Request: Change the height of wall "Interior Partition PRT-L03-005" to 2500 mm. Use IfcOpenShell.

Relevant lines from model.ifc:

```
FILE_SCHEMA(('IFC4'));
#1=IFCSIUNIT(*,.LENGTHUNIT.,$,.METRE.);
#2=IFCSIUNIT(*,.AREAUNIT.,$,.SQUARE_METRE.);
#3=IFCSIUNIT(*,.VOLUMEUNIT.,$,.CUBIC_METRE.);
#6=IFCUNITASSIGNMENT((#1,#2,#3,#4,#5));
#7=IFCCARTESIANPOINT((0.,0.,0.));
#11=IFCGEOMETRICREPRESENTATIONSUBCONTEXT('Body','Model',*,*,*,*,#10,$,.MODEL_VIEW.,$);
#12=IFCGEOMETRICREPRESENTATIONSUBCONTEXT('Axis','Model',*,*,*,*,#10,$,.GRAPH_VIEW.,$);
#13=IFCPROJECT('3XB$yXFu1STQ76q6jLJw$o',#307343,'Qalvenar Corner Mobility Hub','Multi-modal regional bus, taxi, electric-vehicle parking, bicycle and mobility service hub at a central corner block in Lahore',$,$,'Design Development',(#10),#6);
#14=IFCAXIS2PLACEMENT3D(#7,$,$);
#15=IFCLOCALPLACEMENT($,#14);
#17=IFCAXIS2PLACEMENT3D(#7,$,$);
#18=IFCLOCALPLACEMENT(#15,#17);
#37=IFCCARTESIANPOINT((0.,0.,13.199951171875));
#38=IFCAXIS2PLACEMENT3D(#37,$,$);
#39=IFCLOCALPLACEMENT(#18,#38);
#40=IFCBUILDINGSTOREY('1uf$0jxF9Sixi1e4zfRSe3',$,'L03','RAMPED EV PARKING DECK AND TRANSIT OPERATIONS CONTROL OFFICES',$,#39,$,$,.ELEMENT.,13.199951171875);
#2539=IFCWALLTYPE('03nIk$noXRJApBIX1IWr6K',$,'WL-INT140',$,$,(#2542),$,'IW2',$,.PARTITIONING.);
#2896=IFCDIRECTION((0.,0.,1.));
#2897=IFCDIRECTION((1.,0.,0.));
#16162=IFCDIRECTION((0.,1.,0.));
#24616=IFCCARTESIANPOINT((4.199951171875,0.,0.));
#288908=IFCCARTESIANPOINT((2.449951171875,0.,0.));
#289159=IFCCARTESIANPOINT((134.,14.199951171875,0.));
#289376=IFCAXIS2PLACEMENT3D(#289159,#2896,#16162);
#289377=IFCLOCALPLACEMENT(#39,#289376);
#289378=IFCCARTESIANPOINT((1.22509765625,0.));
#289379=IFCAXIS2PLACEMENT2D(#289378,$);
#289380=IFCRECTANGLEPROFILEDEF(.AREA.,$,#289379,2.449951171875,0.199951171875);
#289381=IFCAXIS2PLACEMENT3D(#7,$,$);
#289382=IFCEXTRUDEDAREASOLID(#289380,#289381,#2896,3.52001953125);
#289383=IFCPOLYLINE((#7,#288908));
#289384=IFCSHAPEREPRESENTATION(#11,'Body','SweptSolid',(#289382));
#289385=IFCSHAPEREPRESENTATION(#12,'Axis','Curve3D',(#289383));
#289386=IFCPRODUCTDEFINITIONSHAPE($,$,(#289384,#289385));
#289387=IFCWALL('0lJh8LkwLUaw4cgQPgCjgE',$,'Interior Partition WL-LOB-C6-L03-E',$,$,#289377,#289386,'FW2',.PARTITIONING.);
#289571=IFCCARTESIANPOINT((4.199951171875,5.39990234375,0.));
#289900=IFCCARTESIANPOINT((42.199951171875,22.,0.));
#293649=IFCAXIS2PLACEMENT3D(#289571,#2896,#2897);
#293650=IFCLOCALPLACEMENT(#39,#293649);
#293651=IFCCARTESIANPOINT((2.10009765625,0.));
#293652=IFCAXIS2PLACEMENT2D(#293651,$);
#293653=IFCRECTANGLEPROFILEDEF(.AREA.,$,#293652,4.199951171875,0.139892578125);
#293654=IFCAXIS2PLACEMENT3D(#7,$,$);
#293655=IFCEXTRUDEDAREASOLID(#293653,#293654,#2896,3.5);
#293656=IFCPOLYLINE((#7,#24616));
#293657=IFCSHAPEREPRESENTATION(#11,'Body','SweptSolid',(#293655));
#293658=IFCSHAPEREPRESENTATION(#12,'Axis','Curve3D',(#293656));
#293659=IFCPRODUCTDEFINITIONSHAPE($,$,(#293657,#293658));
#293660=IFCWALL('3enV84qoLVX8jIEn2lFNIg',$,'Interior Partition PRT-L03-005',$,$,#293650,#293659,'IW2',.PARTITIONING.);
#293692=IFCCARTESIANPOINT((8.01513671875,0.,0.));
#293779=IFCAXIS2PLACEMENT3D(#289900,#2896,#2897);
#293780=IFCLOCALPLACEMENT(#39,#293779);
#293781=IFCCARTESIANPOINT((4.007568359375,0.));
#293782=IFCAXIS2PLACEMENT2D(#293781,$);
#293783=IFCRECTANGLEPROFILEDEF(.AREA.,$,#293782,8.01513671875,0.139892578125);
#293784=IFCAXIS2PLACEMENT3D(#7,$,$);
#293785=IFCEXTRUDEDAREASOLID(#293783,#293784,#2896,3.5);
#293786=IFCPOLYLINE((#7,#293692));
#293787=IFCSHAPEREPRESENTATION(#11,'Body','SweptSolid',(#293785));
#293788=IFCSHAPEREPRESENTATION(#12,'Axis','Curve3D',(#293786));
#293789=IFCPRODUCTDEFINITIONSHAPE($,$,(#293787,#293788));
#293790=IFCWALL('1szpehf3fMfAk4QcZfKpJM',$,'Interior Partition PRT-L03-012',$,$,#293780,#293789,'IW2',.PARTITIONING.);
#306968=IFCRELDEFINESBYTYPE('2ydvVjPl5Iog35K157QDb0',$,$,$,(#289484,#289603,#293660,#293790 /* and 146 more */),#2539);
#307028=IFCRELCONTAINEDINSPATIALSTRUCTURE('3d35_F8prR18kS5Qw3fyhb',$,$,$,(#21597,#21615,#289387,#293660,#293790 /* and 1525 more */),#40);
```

```python
import ifcopenshell
import ifcopenshell.geom
import ifcopenshell.util.representation
import ifcopenshell.util.shape
import ifcopenshell.util.unit

model = ifcopenshell.open("model.ifc")
unit_scale = ifcopenshell.util.unit.calculate_unit_scale(model)
settings = ifcopenshell.geom.settings()


def volume(element):
    """Net volume in cubic metres, openings subtracted."""
    shape = ifcopenshell.geom.create_shape(settings, element)
    return ifcopenshell.util.shape.get_volume(shape.geometry)


wall = model.by_guid("3enV84qoLVX8jIEn2lFNIg")
before = volume(wall)

body = ifcopenshell.util.representation.get_representation(wall, "Model", "Body")
solid = body.Items[0]
old_height = solid.Depth
solid.Depth = 2.5 / unit_scale
after = volume(wall)

print(f"height {old_height:g} -> {solid.Depth:g}, volume {before:.3f} -> {after:.3f} m3")

model.write("model_edited.ifc")
```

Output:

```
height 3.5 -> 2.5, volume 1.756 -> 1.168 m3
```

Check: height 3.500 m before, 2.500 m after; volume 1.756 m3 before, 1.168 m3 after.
